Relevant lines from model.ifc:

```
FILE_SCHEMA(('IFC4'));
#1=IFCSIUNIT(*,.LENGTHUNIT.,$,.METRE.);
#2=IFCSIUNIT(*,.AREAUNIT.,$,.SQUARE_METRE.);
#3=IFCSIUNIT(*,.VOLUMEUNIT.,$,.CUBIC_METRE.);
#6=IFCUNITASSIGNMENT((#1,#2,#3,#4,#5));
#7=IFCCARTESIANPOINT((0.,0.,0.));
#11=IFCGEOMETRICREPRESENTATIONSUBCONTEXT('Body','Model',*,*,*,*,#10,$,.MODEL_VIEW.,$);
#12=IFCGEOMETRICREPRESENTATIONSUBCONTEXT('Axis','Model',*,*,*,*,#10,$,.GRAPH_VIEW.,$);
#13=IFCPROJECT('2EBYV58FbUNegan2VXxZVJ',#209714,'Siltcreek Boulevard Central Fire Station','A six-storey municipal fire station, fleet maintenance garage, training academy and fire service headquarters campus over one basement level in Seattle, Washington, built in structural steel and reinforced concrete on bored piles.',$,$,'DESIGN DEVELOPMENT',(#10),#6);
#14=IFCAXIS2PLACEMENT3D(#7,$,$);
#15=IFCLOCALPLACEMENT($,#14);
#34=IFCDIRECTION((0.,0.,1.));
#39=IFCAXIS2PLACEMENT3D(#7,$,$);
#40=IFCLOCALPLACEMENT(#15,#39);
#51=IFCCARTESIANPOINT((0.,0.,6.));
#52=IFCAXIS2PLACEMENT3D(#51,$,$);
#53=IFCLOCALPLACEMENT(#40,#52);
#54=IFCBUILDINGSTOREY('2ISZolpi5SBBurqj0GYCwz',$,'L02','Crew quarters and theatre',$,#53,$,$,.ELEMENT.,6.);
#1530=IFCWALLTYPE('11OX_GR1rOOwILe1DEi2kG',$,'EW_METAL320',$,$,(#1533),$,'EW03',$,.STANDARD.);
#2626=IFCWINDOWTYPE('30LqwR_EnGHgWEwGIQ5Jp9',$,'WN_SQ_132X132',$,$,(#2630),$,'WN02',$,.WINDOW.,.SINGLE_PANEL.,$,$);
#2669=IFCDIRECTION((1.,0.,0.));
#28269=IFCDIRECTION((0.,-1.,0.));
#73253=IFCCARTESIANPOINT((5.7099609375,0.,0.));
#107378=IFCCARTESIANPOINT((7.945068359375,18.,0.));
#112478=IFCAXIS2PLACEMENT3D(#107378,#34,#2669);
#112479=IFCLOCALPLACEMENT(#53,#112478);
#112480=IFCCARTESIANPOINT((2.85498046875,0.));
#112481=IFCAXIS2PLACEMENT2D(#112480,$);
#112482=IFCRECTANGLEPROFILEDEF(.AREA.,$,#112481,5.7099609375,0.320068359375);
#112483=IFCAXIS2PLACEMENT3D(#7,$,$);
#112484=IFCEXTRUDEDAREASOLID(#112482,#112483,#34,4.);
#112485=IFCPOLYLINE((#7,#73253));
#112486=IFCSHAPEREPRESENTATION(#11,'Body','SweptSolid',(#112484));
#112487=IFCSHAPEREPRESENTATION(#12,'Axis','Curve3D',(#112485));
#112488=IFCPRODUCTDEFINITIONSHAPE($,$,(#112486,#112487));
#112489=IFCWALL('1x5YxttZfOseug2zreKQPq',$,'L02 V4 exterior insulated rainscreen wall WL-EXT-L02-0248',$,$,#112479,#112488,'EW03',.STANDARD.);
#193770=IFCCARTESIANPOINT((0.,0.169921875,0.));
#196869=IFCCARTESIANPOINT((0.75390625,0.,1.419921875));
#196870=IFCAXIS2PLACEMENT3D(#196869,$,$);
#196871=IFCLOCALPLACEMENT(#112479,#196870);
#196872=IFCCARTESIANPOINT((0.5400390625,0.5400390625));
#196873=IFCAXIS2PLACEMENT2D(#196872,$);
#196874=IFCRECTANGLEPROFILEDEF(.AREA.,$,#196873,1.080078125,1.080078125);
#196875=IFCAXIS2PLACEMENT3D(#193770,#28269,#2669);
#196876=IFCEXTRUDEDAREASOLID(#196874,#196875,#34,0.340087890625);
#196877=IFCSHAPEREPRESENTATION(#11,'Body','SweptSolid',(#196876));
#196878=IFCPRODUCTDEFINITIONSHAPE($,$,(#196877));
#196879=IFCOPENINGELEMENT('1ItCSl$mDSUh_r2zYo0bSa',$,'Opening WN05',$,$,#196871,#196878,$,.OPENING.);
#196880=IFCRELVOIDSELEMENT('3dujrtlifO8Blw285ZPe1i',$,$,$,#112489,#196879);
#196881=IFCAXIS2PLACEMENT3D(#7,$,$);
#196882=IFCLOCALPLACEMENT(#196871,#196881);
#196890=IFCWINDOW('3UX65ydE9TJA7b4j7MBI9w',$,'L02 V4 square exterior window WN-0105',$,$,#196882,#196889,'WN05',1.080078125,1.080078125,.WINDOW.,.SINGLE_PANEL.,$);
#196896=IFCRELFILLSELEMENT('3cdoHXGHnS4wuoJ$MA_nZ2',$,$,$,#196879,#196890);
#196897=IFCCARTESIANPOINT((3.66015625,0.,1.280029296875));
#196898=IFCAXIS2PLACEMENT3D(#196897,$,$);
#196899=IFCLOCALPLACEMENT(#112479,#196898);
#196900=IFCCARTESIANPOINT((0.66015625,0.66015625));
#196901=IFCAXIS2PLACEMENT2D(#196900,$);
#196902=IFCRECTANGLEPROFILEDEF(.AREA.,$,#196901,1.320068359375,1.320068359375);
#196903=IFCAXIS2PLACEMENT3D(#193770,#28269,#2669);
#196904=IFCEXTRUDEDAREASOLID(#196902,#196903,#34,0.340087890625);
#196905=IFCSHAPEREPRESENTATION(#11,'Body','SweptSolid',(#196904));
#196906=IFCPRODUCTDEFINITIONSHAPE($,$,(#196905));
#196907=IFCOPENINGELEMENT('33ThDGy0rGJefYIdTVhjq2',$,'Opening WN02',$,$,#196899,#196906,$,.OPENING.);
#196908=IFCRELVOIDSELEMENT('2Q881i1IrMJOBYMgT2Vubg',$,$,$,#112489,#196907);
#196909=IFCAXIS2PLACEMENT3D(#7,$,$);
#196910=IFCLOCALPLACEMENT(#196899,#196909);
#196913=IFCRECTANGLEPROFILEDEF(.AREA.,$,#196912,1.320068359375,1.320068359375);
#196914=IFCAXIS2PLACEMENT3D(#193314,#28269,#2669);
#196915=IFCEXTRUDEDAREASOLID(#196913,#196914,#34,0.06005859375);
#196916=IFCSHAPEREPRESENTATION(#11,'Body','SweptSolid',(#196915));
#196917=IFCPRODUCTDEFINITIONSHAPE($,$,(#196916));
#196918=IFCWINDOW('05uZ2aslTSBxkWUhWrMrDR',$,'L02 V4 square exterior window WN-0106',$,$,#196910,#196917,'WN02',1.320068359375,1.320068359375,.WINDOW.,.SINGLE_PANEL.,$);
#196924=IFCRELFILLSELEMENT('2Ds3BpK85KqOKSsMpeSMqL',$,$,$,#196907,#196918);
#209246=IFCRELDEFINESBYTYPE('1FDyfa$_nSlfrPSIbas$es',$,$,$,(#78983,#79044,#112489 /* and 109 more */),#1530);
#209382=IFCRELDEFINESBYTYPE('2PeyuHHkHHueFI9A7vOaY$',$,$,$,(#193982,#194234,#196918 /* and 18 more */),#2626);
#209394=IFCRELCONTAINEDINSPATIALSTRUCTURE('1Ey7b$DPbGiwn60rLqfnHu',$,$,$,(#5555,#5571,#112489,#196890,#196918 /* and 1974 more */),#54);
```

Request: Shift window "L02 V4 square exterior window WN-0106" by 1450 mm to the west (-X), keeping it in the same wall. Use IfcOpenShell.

```python
import ifcopenshell
import ifcopenshell.api.geometry
import ifcopenshell.util.placement
import ifcopenshell.util.unit

model = ifcopenshell.open("model.ifc")
unit_scale = ifcopenshell.util.unit.calculate_unit_scale(model)

window = model.by_guid("05uZ2aslTSBxkWUhWrMrDR")
opening = window.FillsVoids[0].RelatingOpeningElement
wall = opening.VoidsElements[0].RelatingBuildingElement

wall_matrix = ifcopenshell.util.placement.get_local_placement(wall.ObjectPlacement)
shift = wall_matrix[:3, 0] * -1.45 / unit_scale
before = ifcopenshell.util.placement.get_local_placement(window.ObjectPlacement)[:3, 3].copy()

# The window is placed relative to its opening, so it follows when the opening moves.
matrix = ifcopenshell.util.placement.get_local_placement(opening.ObjectPlacement)
matrix[:3, 3] += shift
ifcopenshell.api.geometry.edit_object_placement(
    model, product=opening, matrix=matrix, is_si=False, should_transform_children=True
)

after = ifcopenshell.util.placement.get_local_placement(window.ObjectPlacement)[:3, 3]
print("window moved by", (after - before).round(3) + 0.0)

model.write("model_v2.ifc")
```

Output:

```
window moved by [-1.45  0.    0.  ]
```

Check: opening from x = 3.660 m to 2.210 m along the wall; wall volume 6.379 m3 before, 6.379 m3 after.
